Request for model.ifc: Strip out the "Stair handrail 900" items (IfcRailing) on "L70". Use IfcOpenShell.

First a look at what the model holds.

```python
import ifcopenshell
import ifcopenshell.util.element

model = ifcopenshell.open("model.ifc")
print(model.schema)
storey = next(s for s in model.by_type("IfcBuildingStorey") if s.Name == "L70")
railings = [e for e in ifcopenshell.util.element.get_decomposition(storey) if e.is_a("IfcRailing")]
seen = {}
for e in railings:
    element_type = ifcopenshell.util.element.get_type(e)
    name = element_type.Name if element_type not in (None, e) else None
    seen[name] = seen.get(name, 0) + 1
for name, count in sorted(seen.items(), key=str):
    print(count, "x", name)
```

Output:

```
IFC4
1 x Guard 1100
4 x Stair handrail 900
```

```python
import ifcopenshell
import ifcopenshell.api.root
import ifcopenshell.util.element

model = ifcopenshell.open("model.ifc")

storey = next(s for s in model.by_type("IfcBuildingStorey") if s.Name == "L70")
railings = [e for e in ifcopenshell.util.element.get_decomposition(storey) if e.is_a("IfcRailing")]
targets = [e for e in railings if (t := ifcopenshell.util.element.get_type(e)) not in (None, e) and t.Name == "Stair handrail 900"]

for e in targets:
    ifcopenshell.api.root.remove_product(model, product=e)
print(len(targets), "removed")

model.write("model-out.ifc")
```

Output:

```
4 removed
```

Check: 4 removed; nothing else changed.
